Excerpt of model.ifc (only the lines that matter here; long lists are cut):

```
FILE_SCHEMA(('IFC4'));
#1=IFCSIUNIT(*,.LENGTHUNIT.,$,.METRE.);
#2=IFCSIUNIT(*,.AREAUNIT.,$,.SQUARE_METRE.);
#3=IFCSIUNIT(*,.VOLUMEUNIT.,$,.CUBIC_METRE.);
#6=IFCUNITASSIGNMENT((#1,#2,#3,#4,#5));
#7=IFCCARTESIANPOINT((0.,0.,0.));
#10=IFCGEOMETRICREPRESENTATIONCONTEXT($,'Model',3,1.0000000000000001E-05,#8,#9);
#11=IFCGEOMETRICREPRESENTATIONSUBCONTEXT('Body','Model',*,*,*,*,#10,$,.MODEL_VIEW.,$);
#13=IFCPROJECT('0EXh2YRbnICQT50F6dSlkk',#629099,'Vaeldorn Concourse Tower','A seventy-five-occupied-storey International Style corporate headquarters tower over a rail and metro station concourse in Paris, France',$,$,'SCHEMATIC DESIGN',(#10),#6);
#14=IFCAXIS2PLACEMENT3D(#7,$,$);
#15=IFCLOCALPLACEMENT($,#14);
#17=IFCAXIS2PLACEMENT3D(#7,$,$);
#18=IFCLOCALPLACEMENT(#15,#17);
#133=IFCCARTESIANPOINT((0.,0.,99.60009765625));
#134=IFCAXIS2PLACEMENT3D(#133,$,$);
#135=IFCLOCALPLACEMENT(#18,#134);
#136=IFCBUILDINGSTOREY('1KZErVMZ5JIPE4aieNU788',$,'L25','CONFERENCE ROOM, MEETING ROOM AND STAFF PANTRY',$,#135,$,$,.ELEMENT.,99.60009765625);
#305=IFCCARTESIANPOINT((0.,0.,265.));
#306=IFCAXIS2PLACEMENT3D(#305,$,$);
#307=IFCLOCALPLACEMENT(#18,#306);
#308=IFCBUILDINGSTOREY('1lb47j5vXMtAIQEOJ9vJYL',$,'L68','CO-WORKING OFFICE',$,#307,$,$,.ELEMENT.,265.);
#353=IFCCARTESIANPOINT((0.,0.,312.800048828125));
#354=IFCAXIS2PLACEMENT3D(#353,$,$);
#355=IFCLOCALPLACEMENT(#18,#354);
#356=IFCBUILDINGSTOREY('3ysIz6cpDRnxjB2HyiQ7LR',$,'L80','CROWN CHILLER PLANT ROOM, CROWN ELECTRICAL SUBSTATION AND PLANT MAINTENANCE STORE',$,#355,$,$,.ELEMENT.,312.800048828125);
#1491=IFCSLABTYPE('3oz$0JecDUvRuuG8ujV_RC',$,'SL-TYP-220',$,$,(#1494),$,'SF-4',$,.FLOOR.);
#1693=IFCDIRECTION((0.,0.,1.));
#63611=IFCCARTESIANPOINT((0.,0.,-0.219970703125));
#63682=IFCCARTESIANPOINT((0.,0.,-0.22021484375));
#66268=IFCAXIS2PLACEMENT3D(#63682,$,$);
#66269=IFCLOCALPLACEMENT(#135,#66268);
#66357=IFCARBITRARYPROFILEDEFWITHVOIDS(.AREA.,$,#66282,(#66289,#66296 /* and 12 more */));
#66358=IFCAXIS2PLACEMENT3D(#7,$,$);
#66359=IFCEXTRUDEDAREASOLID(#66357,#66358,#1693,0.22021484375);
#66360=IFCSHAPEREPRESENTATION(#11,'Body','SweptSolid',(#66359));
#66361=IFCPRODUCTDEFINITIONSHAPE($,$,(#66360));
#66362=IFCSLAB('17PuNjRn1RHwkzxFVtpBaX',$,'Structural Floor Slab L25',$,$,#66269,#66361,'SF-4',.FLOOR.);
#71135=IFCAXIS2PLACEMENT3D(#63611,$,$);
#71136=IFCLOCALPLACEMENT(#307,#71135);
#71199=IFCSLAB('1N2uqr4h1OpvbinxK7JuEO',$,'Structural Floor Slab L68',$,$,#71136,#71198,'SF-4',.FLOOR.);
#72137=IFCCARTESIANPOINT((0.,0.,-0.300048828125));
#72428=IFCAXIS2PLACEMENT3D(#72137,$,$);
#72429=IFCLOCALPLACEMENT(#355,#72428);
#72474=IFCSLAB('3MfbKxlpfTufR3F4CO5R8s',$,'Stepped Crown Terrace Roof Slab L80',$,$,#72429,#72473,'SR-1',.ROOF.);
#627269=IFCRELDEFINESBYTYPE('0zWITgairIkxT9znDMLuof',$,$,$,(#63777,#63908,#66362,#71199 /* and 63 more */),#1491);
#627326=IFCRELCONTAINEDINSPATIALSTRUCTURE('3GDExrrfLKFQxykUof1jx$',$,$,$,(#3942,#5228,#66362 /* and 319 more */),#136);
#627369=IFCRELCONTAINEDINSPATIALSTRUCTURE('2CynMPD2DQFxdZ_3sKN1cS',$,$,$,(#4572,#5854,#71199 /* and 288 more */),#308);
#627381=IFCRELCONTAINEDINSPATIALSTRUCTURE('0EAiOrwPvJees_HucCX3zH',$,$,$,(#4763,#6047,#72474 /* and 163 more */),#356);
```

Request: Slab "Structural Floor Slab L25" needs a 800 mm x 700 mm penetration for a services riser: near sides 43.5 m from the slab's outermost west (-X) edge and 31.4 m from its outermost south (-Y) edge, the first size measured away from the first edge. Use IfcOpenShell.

```python
import numpy as np
import ifcopenshell
import ifcopenshell.api.feature
import ifcopenshell.api.geometry
import ifcopenshell.api.root
import ifcopenshell.geom
import ifcopenshell.util.placement
import ifcopenshell.util.representation
import ifcopenshell.util.shape
import ifcopenshell.util.unit

model = ifcopenshell.open("model.ifc")
unit_scale = ifcopenshell.util.unit.calculate_unit_scale(model)
settings = ifcopenshell.geom.settings()


def volume(element):
    """Net volume in cubic metres, openings subtracted."""
    shape = ifcopenshell.geom.create_shape(settings, element)
    return ifcopenshell.util.shape.get_volume(shape.geometry)


slab = model.by_guid("17PuNjRn1RHwkzxFVtpBaX")
before = volume(slab)

# Extent in the slab's own axes, in metres. The edges named are its -X and -Y sides.
slab_shape = ifcopenshell.geom.create_shape(settings, slab)
vertices = ifcopenshell.util.shape.get_vertices(slab_shape.geometry)
x_min, y_min, bottom = vertices.min(axis=0)
top = vertices[:, 2].max()

opening = ifcopenshell.api.root.create_entity(model, ifc_class="IfcOpeningElement", name="Services riser opening", predefined_type="OPENING")
context = ifcopenshell.util.representation.get_context(model, "Model", "Body", "MODEL_VIEW")
width, depth = 0.8, 0.7
outline = [(0.0, 0.0), (width, 0.0), (width, depth), (0.0, depth), (0.0, 0.0)]
# Overshoot both faces by 50 mm so the cut is clean.
shape = ifcopenshell.api.geometry.add_slab_representation(
    model, context=context, depth=top - bottom + 0.1, polyline=outline
)
ifcopenshell.api.geometry.assign_representation(model, product=opening, representation=shape)

matrix = ifcopenshell.util.placement.get_local_placement(slab.ObjectPlacement)
matrix[:, 3] = matrix @ np.append(np.array([x_min + 43.5, y_min + 31.4, bottom - 0.05]) / unit_scale, 1.0)
ifcopenshell.api.geometry.edit_object_placement(model, product=opening, matrix=matrix, is_si=False)
ifcopenshell.api.feature.add_feature(model, feature=opening, element=slab)

after = volume(slab)

print(f"slab volume {before:.3f} -> {after:.3f} m3")

model.write("model_rev.ifc")
```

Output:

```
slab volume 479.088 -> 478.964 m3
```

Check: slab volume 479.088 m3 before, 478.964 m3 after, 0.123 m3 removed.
